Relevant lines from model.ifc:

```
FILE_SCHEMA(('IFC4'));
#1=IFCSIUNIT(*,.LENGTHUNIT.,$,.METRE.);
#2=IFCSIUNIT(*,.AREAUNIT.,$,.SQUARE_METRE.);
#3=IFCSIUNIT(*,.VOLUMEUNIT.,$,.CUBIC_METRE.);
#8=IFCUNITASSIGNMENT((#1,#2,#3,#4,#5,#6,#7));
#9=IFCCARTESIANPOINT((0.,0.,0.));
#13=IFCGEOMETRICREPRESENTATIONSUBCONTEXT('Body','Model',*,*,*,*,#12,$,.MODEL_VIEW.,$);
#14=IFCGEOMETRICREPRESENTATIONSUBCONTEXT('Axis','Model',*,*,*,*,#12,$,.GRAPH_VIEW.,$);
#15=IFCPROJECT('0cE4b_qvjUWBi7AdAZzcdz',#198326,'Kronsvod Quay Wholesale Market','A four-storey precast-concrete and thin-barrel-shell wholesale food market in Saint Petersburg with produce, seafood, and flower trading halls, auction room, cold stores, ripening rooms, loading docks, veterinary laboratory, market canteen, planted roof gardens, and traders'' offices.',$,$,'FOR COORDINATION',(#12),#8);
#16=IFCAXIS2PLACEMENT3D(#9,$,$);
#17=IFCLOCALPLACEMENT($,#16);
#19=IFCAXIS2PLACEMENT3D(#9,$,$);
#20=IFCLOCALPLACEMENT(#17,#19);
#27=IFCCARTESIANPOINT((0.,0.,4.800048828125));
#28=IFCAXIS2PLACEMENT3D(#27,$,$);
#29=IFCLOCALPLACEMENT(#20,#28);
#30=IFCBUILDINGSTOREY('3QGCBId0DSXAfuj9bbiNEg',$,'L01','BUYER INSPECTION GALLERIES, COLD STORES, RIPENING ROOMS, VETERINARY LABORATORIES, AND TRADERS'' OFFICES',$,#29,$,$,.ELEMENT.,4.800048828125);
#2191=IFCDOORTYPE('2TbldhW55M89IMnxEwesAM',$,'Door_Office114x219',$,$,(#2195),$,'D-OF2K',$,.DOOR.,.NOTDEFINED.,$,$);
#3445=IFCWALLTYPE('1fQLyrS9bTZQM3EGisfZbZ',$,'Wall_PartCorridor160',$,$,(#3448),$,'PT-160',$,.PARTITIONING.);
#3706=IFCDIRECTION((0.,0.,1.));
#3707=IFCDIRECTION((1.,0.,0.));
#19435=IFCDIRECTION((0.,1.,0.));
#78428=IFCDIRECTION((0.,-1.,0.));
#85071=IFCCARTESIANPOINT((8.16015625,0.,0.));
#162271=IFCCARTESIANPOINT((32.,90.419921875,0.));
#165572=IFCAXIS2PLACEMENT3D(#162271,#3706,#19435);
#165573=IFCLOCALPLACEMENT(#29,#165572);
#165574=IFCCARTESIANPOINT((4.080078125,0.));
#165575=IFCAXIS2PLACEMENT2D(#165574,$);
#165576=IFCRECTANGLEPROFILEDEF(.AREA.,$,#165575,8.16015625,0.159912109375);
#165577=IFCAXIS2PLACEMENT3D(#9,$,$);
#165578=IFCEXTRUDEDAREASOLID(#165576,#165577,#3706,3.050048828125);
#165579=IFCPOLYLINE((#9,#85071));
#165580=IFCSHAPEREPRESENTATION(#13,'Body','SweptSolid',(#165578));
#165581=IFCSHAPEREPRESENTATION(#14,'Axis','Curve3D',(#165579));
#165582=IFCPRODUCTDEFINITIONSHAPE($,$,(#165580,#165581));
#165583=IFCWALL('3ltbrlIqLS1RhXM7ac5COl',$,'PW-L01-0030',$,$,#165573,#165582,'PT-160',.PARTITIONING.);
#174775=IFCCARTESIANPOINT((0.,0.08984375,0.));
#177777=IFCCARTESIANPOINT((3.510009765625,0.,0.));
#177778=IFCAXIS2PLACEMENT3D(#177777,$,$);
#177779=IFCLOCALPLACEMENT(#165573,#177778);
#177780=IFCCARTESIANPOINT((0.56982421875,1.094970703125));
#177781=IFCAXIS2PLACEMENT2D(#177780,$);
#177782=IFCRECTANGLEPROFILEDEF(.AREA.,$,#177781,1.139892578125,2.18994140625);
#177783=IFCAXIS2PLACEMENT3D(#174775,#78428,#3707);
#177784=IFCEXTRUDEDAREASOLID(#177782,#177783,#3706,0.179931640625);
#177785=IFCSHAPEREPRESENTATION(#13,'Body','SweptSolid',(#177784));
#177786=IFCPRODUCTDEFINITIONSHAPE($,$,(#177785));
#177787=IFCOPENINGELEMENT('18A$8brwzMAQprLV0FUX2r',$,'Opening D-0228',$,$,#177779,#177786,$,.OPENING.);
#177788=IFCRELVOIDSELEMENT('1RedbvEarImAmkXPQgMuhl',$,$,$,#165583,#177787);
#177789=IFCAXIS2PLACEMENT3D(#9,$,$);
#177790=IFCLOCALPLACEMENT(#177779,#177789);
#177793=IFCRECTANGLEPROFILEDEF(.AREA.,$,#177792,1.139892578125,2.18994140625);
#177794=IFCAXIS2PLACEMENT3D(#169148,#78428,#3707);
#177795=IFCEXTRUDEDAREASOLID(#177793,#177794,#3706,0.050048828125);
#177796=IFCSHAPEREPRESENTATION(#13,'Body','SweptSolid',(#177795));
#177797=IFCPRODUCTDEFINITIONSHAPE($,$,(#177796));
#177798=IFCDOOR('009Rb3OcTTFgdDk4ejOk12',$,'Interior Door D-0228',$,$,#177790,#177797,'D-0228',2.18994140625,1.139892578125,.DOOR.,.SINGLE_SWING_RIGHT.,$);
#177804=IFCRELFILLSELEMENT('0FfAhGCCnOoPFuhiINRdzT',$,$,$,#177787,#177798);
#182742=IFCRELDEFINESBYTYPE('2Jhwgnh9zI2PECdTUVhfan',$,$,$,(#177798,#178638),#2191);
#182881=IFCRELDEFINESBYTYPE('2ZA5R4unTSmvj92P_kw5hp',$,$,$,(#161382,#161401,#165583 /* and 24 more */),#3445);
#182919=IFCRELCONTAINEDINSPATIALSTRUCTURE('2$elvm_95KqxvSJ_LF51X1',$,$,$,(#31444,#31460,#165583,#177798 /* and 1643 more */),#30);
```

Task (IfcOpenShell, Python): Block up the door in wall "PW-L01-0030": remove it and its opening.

```python
import ifcopenshell
import ifcopenshell.api.feature
import ifcopenshell.api.root
import ifcopenshell.geom
import ifcopenshell.util.shape

model = ifcopenshell.open("model.ifc")
settings = ifcopenshell.geom.settings()


def volume(element):
    """Net volume in cubic metres, openings subtracted."""
    shape = ifcopenshell.geom.create_shape(settings, element)
    return ifcopenshell.util.shape.get_volume(shape.geometry)


door = model.by_guid("009Rb3OcTTFgdDk4ejOk12")
opening = door.FillsVoids[0].RelatingOpeningElement
wall = opening.VoidsElements[0].RelatingBuildingElement
before = volume(wall)

ifcopenshell.api.root.remove_product(model, product=door)
ifcopenshell.api.feature.remove_feature(model, feature=opening)

after = volume(wall)

print(f"wall volume {before:.3f} -> {after:.3f} m3")

model.write("model_edited.ifc")
```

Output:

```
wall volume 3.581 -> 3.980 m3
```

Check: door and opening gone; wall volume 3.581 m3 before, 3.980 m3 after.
